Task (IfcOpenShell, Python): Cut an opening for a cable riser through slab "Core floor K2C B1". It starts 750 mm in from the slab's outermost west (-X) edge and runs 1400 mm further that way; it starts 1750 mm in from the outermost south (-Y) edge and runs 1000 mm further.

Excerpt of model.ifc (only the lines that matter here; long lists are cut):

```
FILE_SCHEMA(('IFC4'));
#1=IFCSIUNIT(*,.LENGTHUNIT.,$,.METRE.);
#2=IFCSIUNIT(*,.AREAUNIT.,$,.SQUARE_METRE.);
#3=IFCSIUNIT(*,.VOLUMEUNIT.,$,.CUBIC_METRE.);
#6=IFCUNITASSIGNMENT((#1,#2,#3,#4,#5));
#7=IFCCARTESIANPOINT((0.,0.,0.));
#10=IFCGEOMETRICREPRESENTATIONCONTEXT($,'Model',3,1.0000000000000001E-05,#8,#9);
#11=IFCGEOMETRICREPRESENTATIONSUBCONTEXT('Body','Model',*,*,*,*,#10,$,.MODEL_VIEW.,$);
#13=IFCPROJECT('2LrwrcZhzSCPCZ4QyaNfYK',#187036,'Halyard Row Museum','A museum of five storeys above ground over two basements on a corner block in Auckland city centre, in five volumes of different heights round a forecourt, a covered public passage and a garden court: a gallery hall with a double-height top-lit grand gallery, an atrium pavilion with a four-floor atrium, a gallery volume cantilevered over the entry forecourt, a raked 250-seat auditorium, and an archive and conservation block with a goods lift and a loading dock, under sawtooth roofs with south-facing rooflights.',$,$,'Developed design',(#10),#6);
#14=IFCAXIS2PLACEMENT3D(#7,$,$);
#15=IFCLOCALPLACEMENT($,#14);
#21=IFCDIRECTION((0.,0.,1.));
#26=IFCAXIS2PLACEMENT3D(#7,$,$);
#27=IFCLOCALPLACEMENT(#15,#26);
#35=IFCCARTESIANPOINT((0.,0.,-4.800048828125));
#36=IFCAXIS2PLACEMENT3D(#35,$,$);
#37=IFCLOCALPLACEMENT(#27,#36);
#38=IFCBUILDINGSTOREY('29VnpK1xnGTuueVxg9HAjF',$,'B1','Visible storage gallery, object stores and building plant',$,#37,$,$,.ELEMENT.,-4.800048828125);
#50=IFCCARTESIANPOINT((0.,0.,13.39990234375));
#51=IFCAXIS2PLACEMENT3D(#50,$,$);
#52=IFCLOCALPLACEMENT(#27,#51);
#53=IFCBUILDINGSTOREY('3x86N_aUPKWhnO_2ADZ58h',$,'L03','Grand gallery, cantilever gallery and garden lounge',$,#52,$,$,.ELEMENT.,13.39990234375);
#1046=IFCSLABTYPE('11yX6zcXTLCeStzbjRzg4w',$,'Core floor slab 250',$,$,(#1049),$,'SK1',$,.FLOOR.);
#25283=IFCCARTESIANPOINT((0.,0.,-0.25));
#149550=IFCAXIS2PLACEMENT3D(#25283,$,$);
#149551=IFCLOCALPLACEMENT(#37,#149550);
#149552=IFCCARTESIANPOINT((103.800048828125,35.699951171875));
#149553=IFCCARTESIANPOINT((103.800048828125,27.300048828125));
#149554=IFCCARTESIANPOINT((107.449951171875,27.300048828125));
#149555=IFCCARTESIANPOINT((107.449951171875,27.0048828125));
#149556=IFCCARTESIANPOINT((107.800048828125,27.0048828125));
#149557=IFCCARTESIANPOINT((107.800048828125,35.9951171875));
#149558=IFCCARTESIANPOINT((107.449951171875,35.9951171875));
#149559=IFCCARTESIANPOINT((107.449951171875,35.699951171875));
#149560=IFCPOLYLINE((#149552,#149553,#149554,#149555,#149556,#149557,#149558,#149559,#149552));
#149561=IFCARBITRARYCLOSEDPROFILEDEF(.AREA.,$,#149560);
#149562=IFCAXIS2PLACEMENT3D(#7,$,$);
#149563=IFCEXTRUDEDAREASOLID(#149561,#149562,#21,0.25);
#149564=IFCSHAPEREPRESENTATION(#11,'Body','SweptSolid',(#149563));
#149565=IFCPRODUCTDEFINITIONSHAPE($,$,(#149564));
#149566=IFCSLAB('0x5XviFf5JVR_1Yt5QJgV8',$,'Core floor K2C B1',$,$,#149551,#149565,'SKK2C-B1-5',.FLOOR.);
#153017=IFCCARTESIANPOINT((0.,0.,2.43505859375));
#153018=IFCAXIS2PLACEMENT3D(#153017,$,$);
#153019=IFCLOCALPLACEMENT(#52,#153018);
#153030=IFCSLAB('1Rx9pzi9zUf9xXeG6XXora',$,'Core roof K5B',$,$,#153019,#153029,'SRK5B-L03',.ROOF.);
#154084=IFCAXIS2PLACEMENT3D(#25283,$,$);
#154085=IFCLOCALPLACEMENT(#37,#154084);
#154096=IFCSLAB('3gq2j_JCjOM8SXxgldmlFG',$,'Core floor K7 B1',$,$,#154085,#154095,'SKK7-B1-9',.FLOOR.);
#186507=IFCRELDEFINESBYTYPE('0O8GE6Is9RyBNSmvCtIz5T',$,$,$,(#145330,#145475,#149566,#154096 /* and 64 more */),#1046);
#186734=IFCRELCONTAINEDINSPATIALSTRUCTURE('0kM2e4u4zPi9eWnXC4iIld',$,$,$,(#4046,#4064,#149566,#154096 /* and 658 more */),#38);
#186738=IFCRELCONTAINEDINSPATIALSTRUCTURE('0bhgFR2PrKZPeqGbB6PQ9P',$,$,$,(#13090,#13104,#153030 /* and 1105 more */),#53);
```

```python
import numpy as np
import ifcopenshell
import ifcopenshell.api.feature
import ifcopenshell.api.geometry
import ifcopenshell.api.root
import ifcopenshell.geom
import ifcopenshell.util.placement
import ifcopenshell.util.representation
import ifcopenshell.util.shape
import ifcopenshell.util.unit

model = ifcopenshell.open("model.ifc")
unit_scale = ifcopenshell.util.unit.calculate_unit_scale(model)
settings = ifcopenshell.geom.settings()


def volume(element):
    """Net volume in cubic metres, openings subtracted."""
    shape = ifcopenshell.geom.create_shape(settings, element)
    return ifcopenshell.util.shape.get_volume(shape.geometry)


slab = model.by_guid("0x5XviFf5JVR_1Yt5QJgV8")
before = volume(slab)

# Extent in the slab's own axes, in metres. The edges named are its -X and -Y sides.
slab_shape = ifcopenshell.geom.create_shape(settings, slab)
vertices = ifcopenshell.util.shape.get_vertices(slab_shape.geometry)
x_min, y_min, bottom = vertices.min(axis=0)
top = vertices[:, 2].max()

opening = ifcopenshell.api.root.create_entity(model, ifc_class="IfcOpeningElement", name="Cable riser opening", predefined_type="OPENING")
context = ifcopenshell.util.representation.get_context(model, "Model", "Body", "MODEL_VIEW")
width, depth = 1.4, 1
outline = [(0.0, 0.0), (width, 0.0), (width, depth), (0.0, depth), (0.0, 0.0)]
# Overshoot both faces by 50 mm so the cut is clean.
shape = ifcopenshell.api.geometry.add_slab_representation(
    model, context=context, depth=top - bottom + 0.1, polyline=outline
)
ifcopenshell.api.geometry.assign_representation(model, product=opening, representation=shape)

matrix = ifcopenshell.util.placement.get_local_placement(slab.ObjectPlacement)
matrix[:, 3] = matrix @ np.append(np.array([x_min + 0.75, y_min + 1.75, bottom - 0.05]) / unit_scale, 1.0)
ifcopenshell.api.geometry.edit_object_placement(model, product=opening, matrix=matrix, is_si=False)
ifcopenshell.api.feature.add_feature(model, feature=opening, element=slab)

after = volume(slab)

print(f"slab volume {before:.3f} -> {after:.3f} m3")

model.write("model_rev.ifc")
```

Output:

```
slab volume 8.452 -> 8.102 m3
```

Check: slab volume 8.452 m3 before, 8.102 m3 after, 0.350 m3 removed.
